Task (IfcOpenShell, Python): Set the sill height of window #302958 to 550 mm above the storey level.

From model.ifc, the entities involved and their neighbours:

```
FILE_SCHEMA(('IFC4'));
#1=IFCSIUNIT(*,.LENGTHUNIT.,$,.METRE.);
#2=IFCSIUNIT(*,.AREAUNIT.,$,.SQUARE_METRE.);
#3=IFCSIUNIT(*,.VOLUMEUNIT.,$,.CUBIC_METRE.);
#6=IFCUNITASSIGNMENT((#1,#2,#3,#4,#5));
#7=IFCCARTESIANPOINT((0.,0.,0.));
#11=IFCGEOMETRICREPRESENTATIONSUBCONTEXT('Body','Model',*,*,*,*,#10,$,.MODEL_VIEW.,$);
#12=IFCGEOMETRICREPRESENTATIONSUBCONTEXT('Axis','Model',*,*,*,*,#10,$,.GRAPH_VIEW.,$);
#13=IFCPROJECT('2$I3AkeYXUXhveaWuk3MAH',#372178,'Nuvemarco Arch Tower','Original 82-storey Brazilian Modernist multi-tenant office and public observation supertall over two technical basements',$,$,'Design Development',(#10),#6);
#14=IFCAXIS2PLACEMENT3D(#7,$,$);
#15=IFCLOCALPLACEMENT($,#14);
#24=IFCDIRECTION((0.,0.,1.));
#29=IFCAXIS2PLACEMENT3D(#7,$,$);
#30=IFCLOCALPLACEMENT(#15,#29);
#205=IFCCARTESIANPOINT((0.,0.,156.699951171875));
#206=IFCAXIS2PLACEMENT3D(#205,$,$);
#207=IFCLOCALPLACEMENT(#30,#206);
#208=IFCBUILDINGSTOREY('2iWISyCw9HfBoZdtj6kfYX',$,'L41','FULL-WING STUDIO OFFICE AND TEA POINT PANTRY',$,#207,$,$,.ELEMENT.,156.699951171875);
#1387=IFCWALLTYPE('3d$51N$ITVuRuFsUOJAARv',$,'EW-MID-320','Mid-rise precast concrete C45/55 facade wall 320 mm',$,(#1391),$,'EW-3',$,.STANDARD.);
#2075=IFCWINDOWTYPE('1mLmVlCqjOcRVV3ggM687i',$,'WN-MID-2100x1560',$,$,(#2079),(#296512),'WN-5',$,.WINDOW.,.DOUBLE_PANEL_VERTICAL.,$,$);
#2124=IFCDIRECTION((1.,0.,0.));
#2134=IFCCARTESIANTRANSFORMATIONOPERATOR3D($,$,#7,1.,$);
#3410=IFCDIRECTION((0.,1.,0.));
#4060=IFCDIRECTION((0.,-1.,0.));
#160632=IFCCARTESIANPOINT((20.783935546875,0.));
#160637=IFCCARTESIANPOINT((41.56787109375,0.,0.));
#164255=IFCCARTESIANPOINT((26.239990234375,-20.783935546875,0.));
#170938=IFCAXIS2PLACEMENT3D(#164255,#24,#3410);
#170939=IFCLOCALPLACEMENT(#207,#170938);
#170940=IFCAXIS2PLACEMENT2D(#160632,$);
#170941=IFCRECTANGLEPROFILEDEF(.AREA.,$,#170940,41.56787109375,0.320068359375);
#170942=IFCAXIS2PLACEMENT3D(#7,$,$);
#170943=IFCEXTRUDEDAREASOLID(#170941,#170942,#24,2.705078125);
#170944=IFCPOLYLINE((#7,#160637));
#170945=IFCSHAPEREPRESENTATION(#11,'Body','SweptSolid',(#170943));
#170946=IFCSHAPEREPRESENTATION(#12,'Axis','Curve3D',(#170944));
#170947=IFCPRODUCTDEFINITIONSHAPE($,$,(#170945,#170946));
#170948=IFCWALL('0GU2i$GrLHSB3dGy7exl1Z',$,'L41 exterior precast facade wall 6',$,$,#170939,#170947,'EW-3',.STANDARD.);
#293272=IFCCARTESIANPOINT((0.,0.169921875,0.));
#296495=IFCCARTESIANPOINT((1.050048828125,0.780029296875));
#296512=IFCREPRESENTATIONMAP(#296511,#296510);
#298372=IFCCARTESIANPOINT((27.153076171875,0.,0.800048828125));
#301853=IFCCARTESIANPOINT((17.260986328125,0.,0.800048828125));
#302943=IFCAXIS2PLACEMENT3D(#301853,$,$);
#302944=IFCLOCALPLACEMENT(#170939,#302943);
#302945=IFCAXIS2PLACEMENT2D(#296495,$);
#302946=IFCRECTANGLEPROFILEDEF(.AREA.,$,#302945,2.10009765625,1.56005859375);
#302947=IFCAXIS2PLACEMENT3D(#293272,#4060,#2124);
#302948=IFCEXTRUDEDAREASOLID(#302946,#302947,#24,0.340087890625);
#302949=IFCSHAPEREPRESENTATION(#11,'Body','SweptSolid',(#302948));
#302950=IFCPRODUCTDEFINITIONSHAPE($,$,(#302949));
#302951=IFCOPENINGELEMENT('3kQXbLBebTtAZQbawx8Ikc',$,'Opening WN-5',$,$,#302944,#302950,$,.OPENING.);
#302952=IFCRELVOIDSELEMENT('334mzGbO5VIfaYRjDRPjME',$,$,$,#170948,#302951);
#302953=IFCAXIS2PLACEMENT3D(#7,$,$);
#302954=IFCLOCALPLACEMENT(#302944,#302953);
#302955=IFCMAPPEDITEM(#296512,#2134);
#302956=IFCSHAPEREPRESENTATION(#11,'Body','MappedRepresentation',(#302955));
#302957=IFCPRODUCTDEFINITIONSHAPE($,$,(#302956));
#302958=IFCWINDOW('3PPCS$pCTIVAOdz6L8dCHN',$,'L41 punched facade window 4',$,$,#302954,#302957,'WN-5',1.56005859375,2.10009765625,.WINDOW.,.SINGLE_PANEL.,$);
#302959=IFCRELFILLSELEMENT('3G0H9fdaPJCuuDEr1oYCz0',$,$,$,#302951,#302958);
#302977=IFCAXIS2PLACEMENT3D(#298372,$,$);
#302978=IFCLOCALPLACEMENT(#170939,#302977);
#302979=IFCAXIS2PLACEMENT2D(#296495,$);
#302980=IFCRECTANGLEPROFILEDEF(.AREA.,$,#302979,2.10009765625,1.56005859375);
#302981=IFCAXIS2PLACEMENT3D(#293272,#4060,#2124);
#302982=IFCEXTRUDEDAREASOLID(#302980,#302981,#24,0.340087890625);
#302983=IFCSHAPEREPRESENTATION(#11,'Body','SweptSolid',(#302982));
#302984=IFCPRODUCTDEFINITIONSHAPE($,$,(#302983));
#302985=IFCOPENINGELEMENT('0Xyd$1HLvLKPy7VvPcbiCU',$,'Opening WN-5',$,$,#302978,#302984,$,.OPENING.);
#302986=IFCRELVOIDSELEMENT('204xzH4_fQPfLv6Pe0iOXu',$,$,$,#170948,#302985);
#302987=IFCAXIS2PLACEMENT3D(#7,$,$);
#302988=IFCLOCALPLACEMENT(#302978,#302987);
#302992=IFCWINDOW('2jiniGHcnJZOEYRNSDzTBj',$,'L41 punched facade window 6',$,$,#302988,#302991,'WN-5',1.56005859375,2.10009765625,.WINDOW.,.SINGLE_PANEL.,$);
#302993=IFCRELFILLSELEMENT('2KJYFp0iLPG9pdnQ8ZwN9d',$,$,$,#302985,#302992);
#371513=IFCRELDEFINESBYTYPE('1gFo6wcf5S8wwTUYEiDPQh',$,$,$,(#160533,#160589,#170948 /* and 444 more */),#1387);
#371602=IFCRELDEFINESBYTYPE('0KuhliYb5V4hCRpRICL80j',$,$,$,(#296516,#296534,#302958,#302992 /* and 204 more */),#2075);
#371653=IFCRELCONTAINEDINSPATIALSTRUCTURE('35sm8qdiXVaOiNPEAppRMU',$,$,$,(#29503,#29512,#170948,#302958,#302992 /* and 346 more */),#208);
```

```python
import numpy as np
import ifcopenshell
import ifcopenshell.api.geometry
import ifcopenshell.geom
import ifcopenshell.util.element
import ifcopenshell.util.placement
import ifcopenshell.util.shape
import ifcopenshell.util.unit

model = ifcopenshell.open("model.ifc")
unit_scale = ifcopenshell.util.unit.calculate_unit_scale(model)

window = model.by_guid("3PPCS$pCTIVAOdz6L8dCHN")
opening = window.FillsVoids[0].RelatingOpeningElement
storey = ifcopenshell.util.element.get_container(window, ifc_class="IfcBuildingStorey")
level = ifcopenshell.util.placement.get_local_placement(storey.ObjectPlacement)[2, 3]

# The opening's origin need not be at the sill, so measure its lowest point.
shape = ifcopenshell.geom.create_shape(ifcopenshell.geom.settings(), opening)
bottom = ifcopenshell.util.shape.get_shape_bottom_elevation(shape, shape.geometry) / unit_scale
dz = level + 0.55 / unit_scale - bottom

shift = np.array([0.0, 0.0, dz])
# The window is placed relative to its opening, so it follows when the opening moves.
matrix = ifcopenshell.util.placement.get_local_placement(opening.ObjectPlacement)
matrix[:3, 3] += shift
ifcopenshell.api.geometry.edit_object_placement(
    model, product=opening, matrix=matrix, is_si=False, should_transform_children=True
)

print(f"moved by {dz * unit_scale:+.3f} m")

model.write("model-out.ifc")
```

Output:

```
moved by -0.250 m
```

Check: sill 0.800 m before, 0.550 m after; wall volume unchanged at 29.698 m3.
